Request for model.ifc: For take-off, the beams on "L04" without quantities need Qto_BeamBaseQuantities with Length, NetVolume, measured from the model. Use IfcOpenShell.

First a look at what the model holds.

```python
import ifcopenshell
import ifcopenshell.util.element
import ifcopenshell.util.unit

model = ifcopenshell.open("model.ifc")
print(model.schema)
for unit_type in ("LENGTHUNIT", "AREAUNIT", "VOLUMEUNIT"):
    print(unit_type, ifcopenshell.util.unit.calculate_unit_scale(model, unit_type))
storey = next(s for s in model.by_type("IfcBuildingStorey") if s.Name == "L04")
beams = [e for e in ifcopenshell.util.element.get_decomposition(storey) if e.is_a("IfcBeam")]
for e in sorted(beams, key=lambda e: e.id()):
    print(e.id(), e.is_a(), e.Name, list(ifcopenshell.util.element.get_psets(e, qtos_only=True)), sep=" | ")
```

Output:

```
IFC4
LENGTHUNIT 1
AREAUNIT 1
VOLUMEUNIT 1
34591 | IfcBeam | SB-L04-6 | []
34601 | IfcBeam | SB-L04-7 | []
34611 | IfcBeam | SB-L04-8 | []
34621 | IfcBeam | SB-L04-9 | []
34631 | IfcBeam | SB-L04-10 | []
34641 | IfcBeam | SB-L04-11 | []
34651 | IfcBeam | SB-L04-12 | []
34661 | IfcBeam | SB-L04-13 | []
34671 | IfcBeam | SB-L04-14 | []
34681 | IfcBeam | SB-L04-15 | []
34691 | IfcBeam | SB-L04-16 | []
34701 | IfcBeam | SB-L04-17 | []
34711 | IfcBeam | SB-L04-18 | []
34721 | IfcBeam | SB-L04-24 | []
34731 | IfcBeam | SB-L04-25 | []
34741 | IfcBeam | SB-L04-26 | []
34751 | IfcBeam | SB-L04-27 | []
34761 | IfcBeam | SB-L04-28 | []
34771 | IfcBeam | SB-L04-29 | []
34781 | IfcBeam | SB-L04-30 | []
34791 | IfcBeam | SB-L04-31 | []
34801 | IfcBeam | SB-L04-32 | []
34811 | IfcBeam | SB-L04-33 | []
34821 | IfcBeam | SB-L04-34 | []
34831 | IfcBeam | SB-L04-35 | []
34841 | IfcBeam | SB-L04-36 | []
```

```python
import ifcopenshell
import ifcopenshell.api.pset
import ifcopenshell.geom
import ifcopenshell.util.element
import ifcopenshell.util.shape
import ifcopenshell.util.unit

model = ifcopenshell.open("model.ifc")
unit_scale = ifcopenshell.util.unit.calculate_unit_scale(model)
volume_scale = ifcopenshell.util.unit.calculate_unit_scale(model, "VOLUMEUNIT")
settings = ifcopenshell.geom.settings()

storey = next(s for s in model.by_type("IfcBuildingStorey") if s.Name == "L04")
beams = [e for e in ifcopenshell.util.element.get_decomposition(storey) if e.is_a("IfcBeam")]

for e in sorted(beams, key=lambda e: e.id()):
    if ifcopenshell.util.element.get_psets(e, qtos_only=True, should_inherit=False):
        continue
    # Geometry comes back in metres, in the element's own axes.
    shape = ifcopenshell.geom.create_shape(settings, e)
    values = {
        "Length": ifcopenshell.util.shape.get_max_xyz(shape.geometry) / unit_scale,
        "NetVolume": ifcopenshell.util.shape.get_volume(shape.geometry) / volume_scale,
    }
    qto = ifcopenshell.api.pset.add_qto(model, product=e, name="Qto_BeamBaseQuantities")
    ifcopenshell.api.pset.edit_qto(model, qto=qto, properties=values)
    print(e.id(), {k: round(v, 3) for k, v in values.items()})

model.write("model_edited.ifc")
```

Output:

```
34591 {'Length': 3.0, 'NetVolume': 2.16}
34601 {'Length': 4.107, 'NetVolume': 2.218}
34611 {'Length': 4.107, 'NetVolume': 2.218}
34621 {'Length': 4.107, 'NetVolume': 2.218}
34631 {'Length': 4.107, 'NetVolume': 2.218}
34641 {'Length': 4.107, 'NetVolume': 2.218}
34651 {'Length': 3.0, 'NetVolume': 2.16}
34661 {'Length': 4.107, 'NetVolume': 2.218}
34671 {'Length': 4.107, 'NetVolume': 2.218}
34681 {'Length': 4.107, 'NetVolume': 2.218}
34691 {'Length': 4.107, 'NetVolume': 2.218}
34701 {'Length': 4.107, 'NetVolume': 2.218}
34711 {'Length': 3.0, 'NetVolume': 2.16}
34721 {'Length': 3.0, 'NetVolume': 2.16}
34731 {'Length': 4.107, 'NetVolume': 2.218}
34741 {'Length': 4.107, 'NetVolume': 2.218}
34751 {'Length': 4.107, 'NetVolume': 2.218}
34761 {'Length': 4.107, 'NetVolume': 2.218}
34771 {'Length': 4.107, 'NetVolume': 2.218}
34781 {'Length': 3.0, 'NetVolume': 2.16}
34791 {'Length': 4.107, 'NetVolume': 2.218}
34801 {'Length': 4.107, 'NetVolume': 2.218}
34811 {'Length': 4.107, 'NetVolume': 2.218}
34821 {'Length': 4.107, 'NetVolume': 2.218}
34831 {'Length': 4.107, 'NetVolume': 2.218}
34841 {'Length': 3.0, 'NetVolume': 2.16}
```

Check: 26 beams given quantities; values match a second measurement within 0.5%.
